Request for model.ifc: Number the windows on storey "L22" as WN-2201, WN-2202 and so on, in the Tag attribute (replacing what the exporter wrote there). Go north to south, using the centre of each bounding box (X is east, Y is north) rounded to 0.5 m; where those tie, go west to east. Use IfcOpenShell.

First a look at what the model holds.

```python
import ifcopenshell
import ifcopenshell.util.element
import ifcopenshell.util.placement

model = ifcopenshell.open("model.ifc")
print(model.schema)
storey = next(s for s in model.by_type("IfcBuildingStorey") if s.Name == "L22")
windows = [e for e in ifcopenshell.util.element.get_decomposition(storey) if e.is_a("IfcWindow")]
for e in sorted(windows, key=lambda e: e.id()):
    origin = ifcopenshell.util.placement.get_local_placement(e.ObjectPlacement)[:3, 3]
    print(e.id(), e.Tag, e.Name, origin.round(2) + 0.0, sep=" | ")
```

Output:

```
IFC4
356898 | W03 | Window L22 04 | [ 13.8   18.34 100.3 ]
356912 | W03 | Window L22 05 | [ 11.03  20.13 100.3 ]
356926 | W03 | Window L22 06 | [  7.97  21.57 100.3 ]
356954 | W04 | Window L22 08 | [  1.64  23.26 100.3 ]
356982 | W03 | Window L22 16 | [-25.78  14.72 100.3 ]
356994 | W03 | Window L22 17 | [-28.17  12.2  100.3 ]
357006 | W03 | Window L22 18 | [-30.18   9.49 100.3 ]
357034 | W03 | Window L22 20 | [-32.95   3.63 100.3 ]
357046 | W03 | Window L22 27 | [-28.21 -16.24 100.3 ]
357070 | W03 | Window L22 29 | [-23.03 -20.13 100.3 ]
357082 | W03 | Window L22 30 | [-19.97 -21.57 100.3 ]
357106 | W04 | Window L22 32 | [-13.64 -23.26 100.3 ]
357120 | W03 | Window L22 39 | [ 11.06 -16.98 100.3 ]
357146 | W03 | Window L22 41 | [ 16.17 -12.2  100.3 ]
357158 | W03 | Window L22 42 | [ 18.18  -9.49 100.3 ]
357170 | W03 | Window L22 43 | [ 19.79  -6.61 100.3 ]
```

```python
import ifcopenshell
import ifcopenshell.geom
import ifcopenshell.util.element
import ifcopenshell.util.shape

model = ifcopenshell.open("model.ifc")
settings = ifcopenshell.geom.settings()
settings.set("use-world-coords", True)


def centre(element):
    shape = ifcopenshell.geom.create_shape(settings, element)
    return ifcopenshell.util.shape.get_bbox_centroid(shape.geometry)


storey = next(s for s in model.by_type("IfcBuildingStorey") if s.Name == "L22")
windows = [e for e in ifcopenshell.util.element.get_decomposition(storey) if e.is_a("IfcWindow")]

# Insertion points can sit at a corner or the storey origin, so sort by the geometry (in metres).
centres = {e: centre(e) for e in windows}
windows.sort(key=lambda e: (-round(centres[e][1] / 0.5), centres[e][0]))

for i, e in enumerate(windows, start=1):
    number = f"WN-22{i:02d}"
    e.Tag = number
    print(e.id(), number)

model.write("model_rev.ifc")
```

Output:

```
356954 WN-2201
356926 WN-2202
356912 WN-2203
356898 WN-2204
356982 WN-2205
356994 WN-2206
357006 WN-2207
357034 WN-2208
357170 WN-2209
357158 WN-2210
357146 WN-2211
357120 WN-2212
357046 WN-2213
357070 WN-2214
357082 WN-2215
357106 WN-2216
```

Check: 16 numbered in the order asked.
